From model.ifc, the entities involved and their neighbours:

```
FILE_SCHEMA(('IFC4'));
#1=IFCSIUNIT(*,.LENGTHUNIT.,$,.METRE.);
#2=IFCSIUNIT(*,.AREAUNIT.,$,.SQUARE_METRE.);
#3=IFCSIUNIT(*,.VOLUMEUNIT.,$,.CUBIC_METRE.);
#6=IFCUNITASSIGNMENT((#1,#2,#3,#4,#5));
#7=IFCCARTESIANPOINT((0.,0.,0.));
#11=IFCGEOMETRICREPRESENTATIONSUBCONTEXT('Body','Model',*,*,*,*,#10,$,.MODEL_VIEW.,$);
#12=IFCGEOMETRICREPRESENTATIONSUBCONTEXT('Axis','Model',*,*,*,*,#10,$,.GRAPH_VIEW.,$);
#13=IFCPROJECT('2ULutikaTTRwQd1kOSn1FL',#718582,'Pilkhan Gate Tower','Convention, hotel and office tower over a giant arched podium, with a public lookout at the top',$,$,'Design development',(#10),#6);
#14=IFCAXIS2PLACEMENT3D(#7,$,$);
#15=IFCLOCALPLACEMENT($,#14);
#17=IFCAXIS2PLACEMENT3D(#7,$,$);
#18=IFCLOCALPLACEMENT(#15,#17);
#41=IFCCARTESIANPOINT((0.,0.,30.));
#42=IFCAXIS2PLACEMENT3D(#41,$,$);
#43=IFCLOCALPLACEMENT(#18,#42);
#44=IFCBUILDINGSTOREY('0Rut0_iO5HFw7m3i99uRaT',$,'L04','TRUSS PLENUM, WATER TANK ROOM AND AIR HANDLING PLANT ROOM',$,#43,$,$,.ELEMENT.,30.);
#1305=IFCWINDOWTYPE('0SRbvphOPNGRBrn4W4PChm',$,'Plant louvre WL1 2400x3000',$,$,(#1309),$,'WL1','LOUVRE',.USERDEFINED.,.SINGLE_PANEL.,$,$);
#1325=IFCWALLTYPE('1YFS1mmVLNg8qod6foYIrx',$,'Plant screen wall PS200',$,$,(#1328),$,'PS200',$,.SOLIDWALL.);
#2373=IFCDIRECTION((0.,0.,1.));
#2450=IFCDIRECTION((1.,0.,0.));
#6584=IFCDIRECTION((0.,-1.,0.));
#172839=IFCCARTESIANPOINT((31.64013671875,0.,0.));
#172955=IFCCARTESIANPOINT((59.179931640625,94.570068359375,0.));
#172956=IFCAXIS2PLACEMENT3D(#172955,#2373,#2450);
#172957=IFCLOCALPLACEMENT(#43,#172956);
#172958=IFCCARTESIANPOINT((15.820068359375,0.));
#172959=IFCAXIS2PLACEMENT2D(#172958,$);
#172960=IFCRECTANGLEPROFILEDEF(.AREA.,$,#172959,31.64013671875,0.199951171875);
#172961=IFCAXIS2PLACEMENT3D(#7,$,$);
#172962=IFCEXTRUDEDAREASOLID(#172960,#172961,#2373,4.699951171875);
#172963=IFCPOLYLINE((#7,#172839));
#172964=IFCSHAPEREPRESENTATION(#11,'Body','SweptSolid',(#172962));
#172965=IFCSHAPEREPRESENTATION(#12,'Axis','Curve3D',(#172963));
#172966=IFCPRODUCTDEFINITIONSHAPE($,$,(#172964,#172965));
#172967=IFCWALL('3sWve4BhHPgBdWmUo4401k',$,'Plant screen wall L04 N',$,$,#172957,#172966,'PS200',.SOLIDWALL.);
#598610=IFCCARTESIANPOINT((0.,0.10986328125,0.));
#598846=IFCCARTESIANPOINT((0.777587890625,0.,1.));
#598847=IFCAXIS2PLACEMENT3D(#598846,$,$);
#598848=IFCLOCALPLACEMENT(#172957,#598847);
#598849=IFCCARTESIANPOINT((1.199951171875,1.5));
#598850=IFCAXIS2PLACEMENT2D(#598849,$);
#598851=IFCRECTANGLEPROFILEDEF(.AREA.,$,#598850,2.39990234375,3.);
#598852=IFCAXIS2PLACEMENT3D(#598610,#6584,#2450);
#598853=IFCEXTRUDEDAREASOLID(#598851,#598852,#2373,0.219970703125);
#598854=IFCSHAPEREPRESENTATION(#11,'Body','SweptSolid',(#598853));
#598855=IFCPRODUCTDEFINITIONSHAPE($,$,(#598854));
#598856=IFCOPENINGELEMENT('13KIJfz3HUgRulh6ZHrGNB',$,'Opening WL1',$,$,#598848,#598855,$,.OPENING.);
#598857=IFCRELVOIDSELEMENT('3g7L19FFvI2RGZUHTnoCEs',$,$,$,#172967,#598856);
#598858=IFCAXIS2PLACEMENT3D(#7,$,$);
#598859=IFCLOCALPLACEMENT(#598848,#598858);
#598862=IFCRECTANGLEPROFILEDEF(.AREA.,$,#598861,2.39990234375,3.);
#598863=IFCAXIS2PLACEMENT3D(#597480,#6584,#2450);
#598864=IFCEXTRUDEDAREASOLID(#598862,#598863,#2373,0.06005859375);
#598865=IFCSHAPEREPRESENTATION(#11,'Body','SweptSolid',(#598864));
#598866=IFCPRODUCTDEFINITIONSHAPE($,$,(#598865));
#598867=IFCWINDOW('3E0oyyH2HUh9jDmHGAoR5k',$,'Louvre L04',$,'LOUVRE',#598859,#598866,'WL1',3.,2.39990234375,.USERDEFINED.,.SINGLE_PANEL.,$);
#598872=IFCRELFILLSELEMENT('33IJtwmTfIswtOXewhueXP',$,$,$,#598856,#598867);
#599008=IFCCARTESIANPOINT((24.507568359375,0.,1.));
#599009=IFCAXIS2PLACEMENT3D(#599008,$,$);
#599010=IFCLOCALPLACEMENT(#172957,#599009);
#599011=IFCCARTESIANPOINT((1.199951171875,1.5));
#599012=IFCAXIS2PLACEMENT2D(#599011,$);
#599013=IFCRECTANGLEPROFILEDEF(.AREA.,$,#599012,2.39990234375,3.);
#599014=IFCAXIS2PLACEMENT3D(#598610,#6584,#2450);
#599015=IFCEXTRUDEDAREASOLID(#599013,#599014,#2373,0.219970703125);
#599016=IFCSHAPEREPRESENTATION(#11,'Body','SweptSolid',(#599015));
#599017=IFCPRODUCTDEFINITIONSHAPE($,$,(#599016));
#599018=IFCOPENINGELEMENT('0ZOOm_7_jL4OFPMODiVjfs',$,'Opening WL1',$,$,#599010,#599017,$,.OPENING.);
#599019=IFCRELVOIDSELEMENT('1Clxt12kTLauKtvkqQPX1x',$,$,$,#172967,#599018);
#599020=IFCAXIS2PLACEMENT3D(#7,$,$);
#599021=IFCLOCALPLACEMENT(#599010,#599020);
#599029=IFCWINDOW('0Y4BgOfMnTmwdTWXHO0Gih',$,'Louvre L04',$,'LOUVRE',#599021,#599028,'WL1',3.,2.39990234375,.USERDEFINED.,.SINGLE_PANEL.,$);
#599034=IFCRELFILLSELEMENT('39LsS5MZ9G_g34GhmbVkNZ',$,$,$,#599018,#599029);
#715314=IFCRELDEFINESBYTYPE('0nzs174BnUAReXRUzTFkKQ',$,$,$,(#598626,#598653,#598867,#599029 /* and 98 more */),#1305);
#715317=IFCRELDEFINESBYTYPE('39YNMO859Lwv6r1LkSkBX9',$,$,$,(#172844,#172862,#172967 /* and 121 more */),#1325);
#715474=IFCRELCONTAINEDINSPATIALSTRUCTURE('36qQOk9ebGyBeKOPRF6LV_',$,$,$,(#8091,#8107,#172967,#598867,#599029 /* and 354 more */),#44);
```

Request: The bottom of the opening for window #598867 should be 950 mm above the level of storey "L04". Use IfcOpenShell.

```python
import numpy as np
import ifcopenshell
import ifcopenshell.api.geometry
import ifcopenshell.geom
import ifcopenshell.util.element
import ifcopenshell.util.placement
import ifcopenshell.util.shape
import ifcopenshell.util.unit

model = ifcopenshell.open("model.ifc")
unit_scale = ifcopenshell.util.unit.calculate_unit_scale(model)

window = model.by_guid("3E0oyyH2HUh9jDmHGAoR5k")
opening = window.FillsVoids[0].RelatingOpeningElement
storey = ifcopenshell.util.element.get_container(window, ifc_class="IfcBuildingStorey")
level = ifcopenshell.util.placement.get_local_placement(storey.ObjectPlacement)[2, 3]

# The opening's origin need not be at the sill, so measure its lowest point.
shape = ifcopenshell.geom.create_shape(ifcopenshell.geom.settings(), opening)
bottom = ifcopenshell.util.shape.get_shape_bottom_elevation(shape, shape.geometry) / unit_scale
dz = level + 0.95 - bottom

shift = np.array([0.0, 0.0, dz])
# The window is placed relative to its opening, so it follows when the opening moves.
matrix = ifcopenshell.util.placement.get_local_placement(opening.ObjectPlacement)
matrix[:3, 3] += shift
ifcopenshell.api.geometry.edit_object_placement(
    model, product=opening, matrix=matrix, is_si=False, should_transform_children=True
)

print(f"moved by {dz * unit_scale:+.3f} m")

model.write("model_edited.ifc")
```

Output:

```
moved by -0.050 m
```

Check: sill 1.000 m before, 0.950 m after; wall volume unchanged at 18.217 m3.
